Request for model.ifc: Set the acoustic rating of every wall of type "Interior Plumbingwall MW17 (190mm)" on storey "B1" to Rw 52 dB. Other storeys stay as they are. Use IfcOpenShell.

First a look at what the model holds.

```python
import ifcopenshell
import ifcopenshell.util.element

model = ifcopenshell.open("model.ifc")
print(model.schema)
storey = next(s for s in model.by_type("IfcBuildingStorey") if s.Name == "B1")
walls = [e for e in ifcopenshell.util.element.get_decomposition(storey) if e.is_a("IfcWall")]
seen = {}
for e in walls:
    element_type = ifcopenshell.util.element.get_type(e)
    key = (element_type.Name if element_type != e and element_type else None, ifcopenshell.util.element.get_pset(e, "Pset_WallCommon", "AcousticRating"))
    seen[key] = seen.get(key, 0) + 1
for (name, value), count in sorted(seen.items(), key=str):
    print(count, "x", name, "|", value)
```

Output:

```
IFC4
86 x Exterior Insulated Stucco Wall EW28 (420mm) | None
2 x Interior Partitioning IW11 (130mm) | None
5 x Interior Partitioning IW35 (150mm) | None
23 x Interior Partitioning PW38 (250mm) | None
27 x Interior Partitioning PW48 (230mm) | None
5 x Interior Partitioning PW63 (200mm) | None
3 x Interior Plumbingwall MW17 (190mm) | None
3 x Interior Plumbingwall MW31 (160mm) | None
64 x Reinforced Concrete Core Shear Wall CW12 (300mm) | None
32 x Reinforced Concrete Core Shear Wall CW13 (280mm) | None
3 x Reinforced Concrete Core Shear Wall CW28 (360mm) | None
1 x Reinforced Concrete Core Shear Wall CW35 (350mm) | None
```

```python
import ifcopenshell
import ifcopenshell.api.pset
import ifcopenshell.util.element

model = ifcopenshell.open("model.ifc")

storey = next(s for s in model.by_type("IfcBuildingStorey") if s.Name == "B1")
walls = [e for e in ifcopenshell.util.element.get_decomposition(storey) if e.is_a("IfcWall")]

count = 0
for e in walls:
    element_type = ifcopenshell.util.element.get_type(e)
    if element_type in (None, e) or element_type.Name != "Interior Plumbingwall MW17 (190mm)":
        continue
    # add_pset returns the element's existing set when there is one.
    pset = ifcopenshell.api.pset.add_pset(model, product=e, name="Pset_WallCommon")
    ifcopenshell.api.pset.edit_pset(model, pset=pset, properties={"AcousticRating": "Rw 52 dB"})
    count += 1

print(count, "walls updated")

model.write("model_v2.ifc")
```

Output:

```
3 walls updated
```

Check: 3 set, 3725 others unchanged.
